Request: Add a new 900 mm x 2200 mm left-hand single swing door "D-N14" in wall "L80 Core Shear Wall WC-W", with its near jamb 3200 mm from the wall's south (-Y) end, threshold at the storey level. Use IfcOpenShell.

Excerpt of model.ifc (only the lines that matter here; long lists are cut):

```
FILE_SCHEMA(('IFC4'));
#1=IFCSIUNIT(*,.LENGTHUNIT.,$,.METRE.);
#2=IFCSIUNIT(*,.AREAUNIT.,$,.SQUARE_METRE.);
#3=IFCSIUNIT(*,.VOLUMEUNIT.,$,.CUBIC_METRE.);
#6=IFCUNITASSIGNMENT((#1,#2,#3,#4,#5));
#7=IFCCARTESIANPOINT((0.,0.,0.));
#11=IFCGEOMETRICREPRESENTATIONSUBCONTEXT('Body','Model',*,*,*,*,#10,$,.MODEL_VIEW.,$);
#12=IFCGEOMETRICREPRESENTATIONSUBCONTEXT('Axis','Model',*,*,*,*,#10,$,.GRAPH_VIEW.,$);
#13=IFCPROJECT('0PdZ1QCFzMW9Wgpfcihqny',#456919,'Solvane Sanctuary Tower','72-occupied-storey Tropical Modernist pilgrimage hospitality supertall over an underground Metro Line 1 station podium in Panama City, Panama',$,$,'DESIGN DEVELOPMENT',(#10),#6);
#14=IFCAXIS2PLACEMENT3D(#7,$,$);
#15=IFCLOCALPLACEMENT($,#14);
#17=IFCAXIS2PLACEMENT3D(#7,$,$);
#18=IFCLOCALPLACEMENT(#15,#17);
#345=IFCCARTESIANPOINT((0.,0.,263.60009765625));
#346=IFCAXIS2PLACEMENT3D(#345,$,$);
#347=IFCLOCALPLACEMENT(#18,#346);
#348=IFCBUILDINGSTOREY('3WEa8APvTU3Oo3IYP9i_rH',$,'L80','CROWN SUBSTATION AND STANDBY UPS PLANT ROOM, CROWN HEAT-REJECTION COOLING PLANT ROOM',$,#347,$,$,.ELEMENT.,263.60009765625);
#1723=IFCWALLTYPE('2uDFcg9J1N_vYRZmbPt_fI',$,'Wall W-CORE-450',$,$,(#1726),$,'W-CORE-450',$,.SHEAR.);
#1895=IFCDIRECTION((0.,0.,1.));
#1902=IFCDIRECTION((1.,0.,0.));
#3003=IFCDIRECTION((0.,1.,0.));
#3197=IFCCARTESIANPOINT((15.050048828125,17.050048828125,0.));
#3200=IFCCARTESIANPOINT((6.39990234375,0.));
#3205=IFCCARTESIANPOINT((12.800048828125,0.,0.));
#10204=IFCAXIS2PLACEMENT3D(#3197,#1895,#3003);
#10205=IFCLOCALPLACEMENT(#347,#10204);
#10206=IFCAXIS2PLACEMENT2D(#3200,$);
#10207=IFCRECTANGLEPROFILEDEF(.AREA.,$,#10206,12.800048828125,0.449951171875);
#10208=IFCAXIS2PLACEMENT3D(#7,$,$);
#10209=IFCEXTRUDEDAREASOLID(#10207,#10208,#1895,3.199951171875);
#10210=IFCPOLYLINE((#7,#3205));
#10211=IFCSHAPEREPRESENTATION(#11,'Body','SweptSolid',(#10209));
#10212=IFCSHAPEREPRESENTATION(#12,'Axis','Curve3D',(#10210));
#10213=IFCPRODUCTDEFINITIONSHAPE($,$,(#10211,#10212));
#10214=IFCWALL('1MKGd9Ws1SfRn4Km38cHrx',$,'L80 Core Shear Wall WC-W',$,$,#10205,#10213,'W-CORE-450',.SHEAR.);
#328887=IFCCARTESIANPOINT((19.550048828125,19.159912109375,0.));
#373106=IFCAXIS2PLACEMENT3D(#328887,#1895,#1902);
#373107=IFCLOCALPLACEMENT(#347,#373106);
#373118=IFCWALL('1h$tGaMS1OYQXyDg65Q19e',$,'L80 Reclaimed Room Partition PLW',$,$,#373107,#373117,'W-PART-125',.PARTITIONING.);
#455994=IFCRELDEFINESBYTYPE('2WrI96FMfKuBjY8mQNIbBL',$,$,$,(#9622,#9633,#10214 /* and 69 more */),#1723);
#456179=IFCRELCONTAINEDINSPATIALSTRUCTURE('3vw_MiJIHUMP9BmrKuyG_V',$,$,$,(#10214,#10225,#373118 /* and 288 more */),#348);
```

```python
import numpy as np
import ifcopenshell
import ifcopenshell.api.feature
import ifcopenshell.api.geometry
import ifcopenshell.api.root
import ifcopenshell.api.spatial
import ifcopenshell.geom
import ifcopenshell.util.element
import ifcopenshell.util.placement
import ifcopenshell.util.representation
import ifcopenshell.util.shape
import ifcopenshell.util.unit

model = ifcopenshell.open("model.ifc")
unit_scale = ifcopenshell.util.unit.calculate_unit_scale(model)
settings = ifcopenshell.geom.settings()


def volume(element):
    """Net volume in cubic metres, openings subtracted."""
    shape = ifcopenshell.geom.create_shape(settings, element)
    return ifcopenshell.util.shape.get_volume(shape.geometry)


wall = model.by_guid("1MKGd9Ws1SfRn4Km38cHrx")
storey = ifcopenshell.util.element.get_container(wall, ifc_class="IfcBuildingStorey")
context = ifcopenshell.util.representation.get_context(model, "Model", "Body", "MODEL_VIEW")
before = volume(wall)

width, height, from_end, sill = 0.9, 2.2, 3.2, 0.0  # metres

# The wall runs along its own X axis, and the end named is its -X end.
wall_shape = ifcopenshell.geom.create_shape(settings, wall)
x, y, z = ifcopenshell.util.shape.get_vertices(wall_shape.geometry).T
start = x.min() + from_end
face, thickness = float(y.min()), float(y.max() - y.min())
wall_matrix = ifcopenshell.util.placement.get_local_placement(wall.ObjectPlacement)
level = ifcopenshell.util.placement.get_local_placement(storey.ObjectPlacement)[2, 3]


def in_wall(x, y):
    """Placement at x, y metres in the wall's axes, at sill height."""
    matrix = wall_matrix.copy()
    matrix[:, 3] = wall_matrix @ np.array([x / unit_scale, y / unit_scale, 0.0, 1.0])
    matrix[2, 3] = level + sill / unit_scale
    return matrix


# Opening: a box that overshoots both wall faces by 50 mm.
opening = ifcopenshell.api.root.create_entity(model, ifc_class="IfcOpeningElement", predefined_type="OPENING")
box = ifcopenshell.api.geometry.add_wall_representation(
    model, context=context, length=width, height=height, thickness=thickness + 0.1
)
ifcopenshell.api.geometry.assign_representation(model, product=opening, representation=box)
ifcopenshell.api.geometry.edit_object_placement(model, product=opening, matrix=in_wall(start, face - 0.05), is_si=False)
ifcopenshell.api.feature.add_feature(model, feature=opening, element=wall)

door = ifcopenshell.api.root.create_entity(model, ifc_class="IfcDoor", name="D-N14", predefined_type="DOOR")
door.OverallWidth, door.OverallHeight = width / unit_scale, height / unit_scale
door.OperationType = "SINGLE_SWING_LEFT"
body = ifcopenshell.api.geometry.add_door_representation(
    model,
    context=context,
    overall_width=door.OverallWidth,
    overall_height=door.OverallHeight,
    operation_type="SINGLE_SWING_LEFT",
    lining_properties={"LiningDepth": thickness / unit_scale, "ThresholdDepth": thickness / unit_scale},
)
ifcopenshell.api.geometry.assign_representation(model, product=door, representation=body)
ifcopenshell.api.spatial.assign_container(model, products=[door], relating_structure=storey)
ifcopenshell.api.feature.add_filling(model, opening=opening, element=door)

# The lining spans the wall, so the door starts at the wall face.
ifcopenshell.api.geometry.edit_object_placement(model, product=door, matrix=in_wall(start, face), is_si=False)

after = volume(wall)

print(f"wall volume {before:.3f} -> {after:.3f} m3")

model.write("model_rev.ifc")
```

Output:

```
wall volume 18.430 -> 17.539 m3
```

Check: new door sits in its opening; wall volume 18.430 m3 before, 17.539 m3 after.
